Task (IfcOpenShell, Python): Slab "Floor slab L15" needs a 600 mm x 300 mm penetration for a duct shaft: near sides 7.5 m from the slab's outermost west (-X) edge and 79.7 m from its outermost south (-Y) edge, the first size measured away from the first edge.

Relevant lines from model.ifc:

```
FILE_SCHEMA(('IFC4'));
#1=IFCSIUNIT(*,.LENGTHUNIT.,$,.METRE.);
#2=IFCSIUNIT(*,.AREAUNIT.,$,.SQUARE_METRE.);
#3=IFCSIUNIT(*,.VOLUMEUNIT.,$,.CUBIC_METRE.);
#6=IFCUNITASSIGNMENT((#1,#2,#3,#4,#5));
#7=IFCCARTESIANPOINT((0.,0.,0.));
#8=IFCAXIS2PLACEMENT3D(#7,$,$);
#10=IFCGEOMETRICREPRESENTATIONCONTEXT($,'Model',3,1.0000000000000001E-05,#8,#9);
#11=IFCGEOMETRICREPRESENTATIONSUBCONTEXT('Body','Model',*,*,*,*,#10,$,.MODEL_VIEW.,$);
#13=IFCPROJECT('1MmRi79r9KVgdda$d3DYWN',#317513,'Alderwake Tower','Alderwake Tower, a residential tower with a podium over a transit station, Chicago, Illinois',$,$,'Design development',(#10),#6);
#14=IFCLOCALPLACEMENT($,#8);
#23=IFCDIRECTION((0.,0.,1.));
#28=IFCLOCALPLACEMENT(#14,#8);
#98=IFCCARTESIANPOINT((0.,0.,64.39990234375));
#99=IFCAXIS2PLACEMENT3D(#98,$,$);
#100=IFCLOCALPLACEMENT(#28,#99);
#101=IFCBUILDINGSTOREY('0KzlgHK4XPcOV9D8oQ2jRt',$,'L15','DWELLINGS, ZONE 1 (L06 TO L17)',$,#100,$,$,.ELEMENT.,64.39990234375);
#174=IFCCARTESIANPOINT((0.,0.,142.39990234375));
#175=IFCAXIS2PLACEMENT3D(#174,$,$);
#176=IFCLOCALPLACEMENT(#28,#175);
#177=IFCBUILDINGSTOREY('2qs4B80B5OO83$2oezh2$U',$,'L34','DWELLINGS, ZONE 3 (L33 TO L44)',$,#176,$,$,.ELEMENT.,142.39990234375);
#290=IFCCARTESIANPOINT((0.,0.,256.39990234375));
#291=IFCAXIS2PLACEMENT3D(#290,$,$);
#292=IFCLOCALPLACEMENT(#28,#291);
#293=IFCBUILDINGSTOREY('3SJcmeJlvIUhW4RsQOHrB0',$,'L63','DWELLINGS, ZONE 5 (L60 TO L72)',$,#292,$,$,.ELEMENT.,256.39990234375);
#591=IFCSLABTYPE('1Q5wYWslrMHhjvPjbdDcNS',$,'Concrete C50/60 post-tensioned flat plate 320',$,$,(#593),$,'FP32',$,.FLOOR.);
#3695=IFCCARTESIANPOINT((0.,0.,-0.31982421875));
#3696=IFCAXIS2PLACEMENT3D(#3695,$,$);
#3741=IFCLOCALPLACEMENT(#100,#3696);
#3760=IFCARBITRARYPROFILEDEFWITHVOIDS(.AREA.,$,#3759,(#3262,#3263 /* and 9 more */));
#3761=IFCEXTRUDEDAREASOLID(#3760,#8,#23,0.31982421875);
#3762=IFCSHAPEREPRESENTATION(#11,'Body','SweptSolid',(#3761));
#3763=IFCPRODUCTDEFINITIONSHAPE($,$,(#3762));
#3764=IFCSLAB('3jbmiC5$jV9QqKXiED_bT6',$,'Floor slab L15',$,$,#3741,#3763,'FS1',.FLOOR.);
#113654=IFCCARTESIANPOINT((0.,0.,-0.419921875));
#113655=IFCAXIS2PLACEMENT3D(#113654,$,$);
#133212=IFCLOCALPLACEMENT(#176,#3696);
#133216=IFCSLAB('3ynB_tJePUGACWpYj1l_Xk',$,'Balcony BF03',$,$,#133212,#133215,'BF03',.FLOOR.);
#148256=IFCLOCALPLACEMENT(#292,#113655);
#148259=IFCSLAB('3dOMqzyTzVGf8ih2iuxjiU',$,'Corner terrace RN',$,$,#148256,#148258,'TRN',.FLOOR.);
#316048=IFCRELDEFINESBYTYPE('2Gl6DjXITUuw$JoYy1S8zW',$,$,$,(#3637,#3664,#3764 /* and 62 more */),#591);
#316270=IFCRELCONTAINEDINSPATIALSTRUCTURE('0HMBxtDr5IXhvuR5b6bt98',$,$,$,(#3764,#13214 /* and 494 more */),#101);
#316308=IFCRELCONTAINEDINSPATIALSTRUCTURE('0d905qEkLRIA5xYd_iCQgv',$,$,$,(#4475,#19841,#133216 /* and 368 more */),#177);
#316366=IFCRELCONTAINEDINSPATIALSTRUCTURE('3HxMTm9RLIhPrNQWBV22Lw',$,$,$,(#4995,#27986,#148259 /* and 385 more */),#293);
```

```python
import numpy as np
import ifcopenshell
import ifcopenshell.api.feature
import ifcopenshell.api.geometry
import ifcopenshell.api.root
import ifcopenshell.geom
import ifcopenshell.util.placement
import ifcopenshell.util.representation
import ifcopenshell.util.shape
import ifcopenshell.util.unit

model = ifcopenshell.open("model.ifc")
unit_scale = ifcopenshell.util.unit.calculate_unit_scale(model)
settings = ifcopenshell.geom.settings()


def volume(element):
    """Net volume in cubic metres, openings subtracted."""
    shape = ifcopenshell.geom.create_shape(settings, element)
    return ifcopenshell.util.shape.get_volume(shape.geometry)


slab = model.by_guid("3jbmiC5$jV9QqKXiED_bT6")
before = volume(slab)

# Extent in the slab's own axes, in metres. The edges named are its -X and -Y sides.
slab_shape = ifcopenshell.geom.create_shape(settings, slab)
vertices = ifcopenshell.util.shape.get_vertices(slab_shape.geometry)
x_min, y_min, bottom = vertices.min(axis=0)
top = vertices[:, 2].max()

opening = ifcopenshell.api.root.create_entity(model, ifc_class="IfcOpeningElement", name="Duct shaft opening", predefined_type="OPENING")
context = ifcopenshell.util.representation.get_context(model, "Model", "Body", "MODEL_VIEW")
width, depth = 0.6, 0.3
outline = [(0.0, 0.0), (width, 0.0), (width, depth), (0.0, depth), (0.0, 0.0)]
# Overshoot both faces by 50 mm so the cut is clean.
shape = ifcopenshell.api.geometry.add_slab_representation(
    model, context=context, depth=top - bottom + 0.1, polyline=outline
)
ifcopenshell.api.geometry.assign_representation(model, product=opening, representation=shape)

matrix = ifcopenshell.util.placement.get_local_placement(slab.ObjectPlacement)
matrix[:, 3] = matrix @ np.append(np.array([x_min + 7.5, y_min + 79.7, bottom - 0.05]) / unit_scale, 1.0)
ifcopenshell.api.geometry.edit_object_placement(model, product=opening, matrix=matrix, is_si=False)
ifcopenshell.api.feature.add_feature(model, feature=opening, element=slab)

after = volume(slab)

print(f"slab volume {before:.3f} -> {after:.3f} m3")

model.write("model_updated.ifc")
```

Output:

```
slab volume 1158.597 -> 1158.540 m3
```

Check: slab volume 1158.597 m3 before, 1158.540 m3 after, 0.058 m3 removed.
